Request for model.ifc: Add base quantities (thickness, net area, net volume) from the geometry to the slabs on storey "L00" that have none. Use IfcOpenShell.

First a look at what the model holds.

```python
import ifcopenshell
import ifcopenshell.util.element
import ifcopenshell.util.unit

model = ifcopenshell.open("model.ifc")
print(model.schema)
for unit_type in ("LENGTHUNIT", "AREAUNIT", "VOLUMEUNIT"):
    print(unit_type, ifcopenshell.util.unit.calculate_unit_scale(model, unit_type))
storey = next(s for s in model.by_type("IfcBuildingStorey") if s.Name == "L00")
slabs = [e for e in ifcopenshell.util.element.get_decomposition(storey) if e.is_a("IfcSlab")]
for e in sorted(slabs, key=lambda e: e.id()):
    print(e.id(), e.is_a(), e.Name, list(ifcopenshell.util.element.get_psets(e, qtos_only=True)), sep=" | ")
```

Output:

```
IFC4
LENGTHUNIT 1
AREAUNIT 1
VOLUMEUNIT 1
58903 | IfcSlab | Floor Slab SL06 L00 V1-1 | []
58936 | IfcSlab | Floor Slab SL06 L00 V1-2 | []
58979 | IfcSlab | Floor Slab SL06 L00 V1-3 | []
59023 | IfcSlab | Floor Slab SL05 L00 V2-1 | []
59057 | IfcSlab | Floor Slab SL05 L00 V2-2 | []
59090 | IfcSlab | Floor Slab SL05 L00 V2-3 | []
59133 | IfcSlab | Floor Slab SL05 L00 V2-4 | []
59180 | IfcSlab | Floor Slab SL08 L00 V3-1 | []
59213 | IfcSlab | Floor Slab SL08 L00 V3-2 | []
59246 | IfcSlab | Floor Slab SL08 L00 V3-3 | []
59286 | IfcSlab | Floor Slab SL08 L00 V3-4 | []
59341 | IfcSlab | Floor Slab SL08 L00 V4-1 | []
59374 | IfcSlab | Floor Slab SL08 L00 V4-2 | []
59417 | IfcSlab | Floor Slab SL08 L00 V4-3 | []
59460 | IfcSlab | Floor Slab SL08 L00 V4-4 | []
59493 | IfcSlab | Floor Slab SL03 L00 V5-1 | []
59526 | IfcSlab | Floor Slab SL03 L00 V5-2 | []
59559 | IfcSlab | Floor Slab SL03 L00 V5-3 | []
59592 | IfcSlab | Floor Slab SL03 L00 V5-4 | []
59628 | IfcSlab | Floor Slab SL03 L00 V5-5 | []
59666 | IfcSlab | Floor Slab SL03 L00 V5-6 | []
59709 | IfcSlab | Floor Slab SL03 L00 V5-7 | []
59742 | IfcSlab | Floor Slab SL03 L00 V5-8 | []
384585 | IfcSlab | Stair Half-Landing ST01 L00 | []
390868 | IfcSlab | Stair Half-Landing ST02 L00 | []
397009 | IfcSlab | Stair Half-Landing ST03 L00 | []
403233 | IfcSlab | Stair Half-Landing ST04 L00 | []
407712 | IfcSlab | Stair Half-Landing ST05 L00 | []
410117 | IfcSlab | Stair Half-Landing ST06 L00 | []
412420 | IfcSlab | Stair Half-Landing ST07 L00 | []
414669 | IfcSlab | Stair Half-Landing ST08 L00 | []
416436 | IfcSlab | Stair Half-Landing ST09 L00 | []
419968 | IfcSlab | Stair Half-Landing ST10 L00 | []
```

```python
import ifcopenshell
import ifcopenshell.api.pset
import ifcopenshell.geom
import ifcopenshell.util.element
import ifcopenshell.util.shape
import ifcopenshell.util.unit

model = ifcopenshell.open("model.ifc")
unit_scale = ifcopenshell.util.unit.calculate_unit_scale(model)
area_scale = ifcopenshell.util.unit.calculate_unit_scale(model, "AREAUNIT")
volume_scale = ifcopenshell.util.unit.calculate_unit_scale(model, "VOLUMEUNIT")
settings = ifcopenshell.geom.settings()

storey = next(s for s in model.by_type("IfcBuildingStorey") if s.Name == "L00")
slabs = [e for e in ifcopenshell.util.element.get_decomposition(storey) if e.is_a("IfcSlab")]

for e in sorted(slabs, key=lambda e: e.id()):
    if ifcopenshell.util.element.get_psets(e, qtos_only=True, should_inherit=False):
        continue
    # Geometry comes back in metres, in the element's own axes.
    shape = ifcopenshell.geom.create_shape(settings, e)
    values = {
        "Width": ifcopenshell.util.shape.get_z(shape.geometry) / unit_scale,
        "NetArea": ifcopenshell.util.shape.get_footprint_area(shape.geometry) / area_scale,
        "NetVolume": ifcopenshell.util.shape.get_volume(shape.geometry) / volume_scale,
    }
    qto = ifcopenshell.api.pset.add_qto(model, product=e, name="Qto_SlabBaseQuantities")
    ifcopenshell.api.pset.edit_qto(model, qto=qto, properties=values)
    print(e.id(), {k: round(v, 3) for k, v in values.items()})

model.write("model_rev.ifc")
```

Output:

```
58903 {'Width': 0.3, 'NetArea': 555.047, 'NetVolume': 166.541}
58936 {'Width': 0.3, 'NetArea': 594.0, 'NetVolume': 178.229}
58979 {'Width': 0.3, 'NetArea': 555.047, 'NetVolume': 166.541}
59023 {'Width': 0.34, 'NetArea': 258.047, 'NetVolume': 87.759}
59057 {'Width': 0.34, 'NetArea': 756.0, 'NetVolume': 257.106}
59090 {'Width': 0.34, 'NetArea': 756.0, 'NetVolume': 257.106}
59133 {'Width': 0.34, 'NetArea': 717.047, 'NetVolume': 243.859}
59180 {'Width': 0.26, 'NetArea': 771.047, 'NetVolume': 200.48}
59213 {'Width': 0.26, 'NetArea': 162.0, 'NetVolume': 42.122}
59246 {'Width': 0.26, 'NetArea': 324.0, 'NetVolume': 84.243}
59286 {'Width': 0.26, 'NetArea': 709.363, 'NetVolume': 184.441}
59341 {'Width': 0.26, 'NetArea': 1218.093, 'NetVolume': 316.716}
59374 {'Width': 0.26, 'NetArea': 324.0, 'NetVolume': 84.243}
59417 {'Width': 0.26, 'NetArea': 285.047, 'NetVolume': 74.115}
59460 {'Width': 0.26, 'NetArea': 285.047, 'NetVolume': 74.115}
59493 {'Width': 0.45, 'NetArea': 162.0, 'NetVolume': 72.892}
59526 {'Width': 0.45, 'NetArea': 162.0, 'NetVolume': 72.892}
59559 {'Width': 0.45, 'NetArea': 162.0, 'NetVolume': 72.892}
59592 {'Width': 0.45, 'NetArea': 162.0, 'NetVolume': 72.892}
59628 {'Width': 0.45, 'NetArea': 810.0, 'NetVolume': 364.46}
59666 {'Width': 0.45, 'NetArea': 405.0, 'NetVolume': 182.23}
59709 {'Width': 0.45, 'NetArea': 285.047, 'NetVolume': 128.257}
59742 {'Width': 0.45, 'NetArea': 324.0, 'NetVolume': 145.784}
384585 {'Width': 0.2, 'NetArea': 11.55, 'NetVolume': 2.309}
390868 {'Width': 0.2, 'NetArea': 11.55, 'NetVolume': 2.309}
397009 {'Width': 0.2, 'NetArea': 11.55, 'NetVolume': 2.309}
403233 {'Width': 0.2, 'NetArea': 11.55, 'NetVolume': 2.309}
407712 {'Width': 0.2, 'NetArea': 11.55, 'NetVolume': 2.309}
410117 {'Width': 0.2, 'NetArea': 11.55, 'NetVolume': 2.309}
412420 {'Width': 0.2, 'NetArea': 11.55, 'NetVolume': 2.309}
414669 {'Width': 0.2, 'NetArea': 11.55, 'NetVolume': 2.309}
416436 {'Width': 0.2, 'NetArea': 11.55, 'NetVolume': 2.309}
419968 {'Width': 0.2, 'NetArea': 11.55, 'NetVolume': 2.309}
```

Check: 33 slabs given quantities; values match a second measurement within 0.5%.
